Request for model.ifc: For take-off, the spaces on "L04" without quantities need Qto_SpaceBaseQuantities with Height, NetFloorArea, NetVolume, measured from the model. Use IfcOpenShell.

First a look at what the model holds.

```python
import ifcopenshell
import ifcopenshell.util.element
import ifcopenshell.util.unit

model = ifcopenshell.open("model.ifc")
print(model.schema)
for unit_type in ("LENGTHUNIT", "AREAUNIT", "VOLUMEUNIT"):
    print(unit_type, ifcopenshell.util.unit.calculate_unit_scale(model, unit_type))
storey = next(s for s in model.by_type("IfcBuildingStorey") if s.Name == "L04")
spaces = [e for e in ifcopenshell.util.element.get_decomposition(storey) if e.is_a("IfcSpace")]
for e in sorted(spaces, key=lambda e: e.id()):
    print(e.id(), e.is_a(), e.Name, list(ifcopenshell.util.element.get_psets(e, qtos_only=True)), sep=" | ")
```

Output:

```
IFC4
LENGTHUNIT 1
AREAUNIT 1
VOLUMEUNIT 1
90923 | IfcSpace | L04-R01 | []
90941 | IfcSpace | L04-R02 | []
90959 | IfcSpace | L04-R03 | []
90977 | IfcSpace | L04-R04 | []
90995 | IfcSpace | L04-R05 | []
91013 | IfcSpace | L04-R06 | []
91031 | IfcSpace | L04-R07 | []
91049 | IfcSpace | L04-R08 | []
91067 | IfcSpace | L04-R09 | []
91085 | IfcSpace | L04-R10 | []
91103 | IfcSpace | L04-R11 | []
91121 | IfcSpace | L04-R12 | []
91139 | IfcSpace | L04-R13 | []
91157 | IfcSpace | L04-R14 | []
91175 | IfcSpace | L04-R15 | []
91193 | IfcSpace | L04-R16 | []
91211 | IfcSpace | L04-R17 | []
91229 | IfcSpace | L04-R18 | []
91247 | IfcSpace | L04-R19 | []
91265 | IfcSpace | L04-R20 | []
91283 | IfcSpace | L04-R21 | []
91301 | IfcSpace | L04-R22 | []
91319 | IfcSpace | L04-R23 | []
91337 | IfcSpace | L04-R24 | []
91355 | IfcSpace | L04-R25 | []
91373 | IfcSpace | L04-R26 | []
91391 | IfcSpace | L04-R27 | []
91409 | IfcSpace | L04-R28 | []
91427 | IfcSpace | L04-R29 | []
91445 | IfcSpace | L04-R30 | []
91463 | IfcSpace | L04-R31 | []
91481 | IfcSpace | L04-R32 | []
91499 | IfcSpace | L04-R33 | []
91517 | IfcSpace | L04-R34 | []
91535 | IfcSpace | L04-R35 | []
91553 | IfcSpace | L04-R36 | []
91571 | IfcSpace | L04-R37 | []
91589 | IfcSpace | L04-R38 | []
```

```python
import ifcopenshell
import ifcopenshell.api.pset
import ifcopenshell.geom
import ifcopenshell.util.element
import ifcopenshell.util.shape
import ifcopenshell.util.unit

model = ifcopenshell.open("model.ifc")
unit_scale = ifcopenshell.util.unit.calculate_unit_scale(model)
area_scale = ifcopenshell.util.unit.calculate_unit_scale(model, "AREAUNIT")
volume_scale = ifcopenshell.util.unit.calculate_unit_scale(model, "VOLUMEUNIT")
settings = ifcopenshell.geom.settings()

storey = next(s for s in model.by_type("IfcBuildingStorey") if s.Name == "L04")
spaces = [e for e in ifcopenshell.util.element.get_decomposition(storey) if e.is_a("IfcSpace")]

for e in sorted(spaces, key=lambda e: e.id()):
    if ifcopenshell.util.element.get_psets(e, qtos_only=True, should_inherit=False):
        continue
    # Geometry comes back in metres, in the element's own axes.
    shape = ifcopenshell.geom.create_shape(settings, e)
    values = {
        "Height": ifcopenshell.util.shape.get_z(shape.geometry) / unit_scale,
        "NetFloorArea": ifcopenshell.util.shape.get_footprint_area(shape.geometry) / area_scale,
        "NetVolume": ifcopenshell.util.shape.get_volume(shape.geometry) / volume_scale,
    }
    qto = ifcopenshell.api.pset.add_qto(model, product=e, name="Qto_SpaceBaseQuantities")
    ifcopenshell.api.pset.edit_qto(model, qto=qto, properties=values)
    print(e.id(), {k: round(v, 3) for k, v in values.items()})

model.write("model_rev.ifc")
```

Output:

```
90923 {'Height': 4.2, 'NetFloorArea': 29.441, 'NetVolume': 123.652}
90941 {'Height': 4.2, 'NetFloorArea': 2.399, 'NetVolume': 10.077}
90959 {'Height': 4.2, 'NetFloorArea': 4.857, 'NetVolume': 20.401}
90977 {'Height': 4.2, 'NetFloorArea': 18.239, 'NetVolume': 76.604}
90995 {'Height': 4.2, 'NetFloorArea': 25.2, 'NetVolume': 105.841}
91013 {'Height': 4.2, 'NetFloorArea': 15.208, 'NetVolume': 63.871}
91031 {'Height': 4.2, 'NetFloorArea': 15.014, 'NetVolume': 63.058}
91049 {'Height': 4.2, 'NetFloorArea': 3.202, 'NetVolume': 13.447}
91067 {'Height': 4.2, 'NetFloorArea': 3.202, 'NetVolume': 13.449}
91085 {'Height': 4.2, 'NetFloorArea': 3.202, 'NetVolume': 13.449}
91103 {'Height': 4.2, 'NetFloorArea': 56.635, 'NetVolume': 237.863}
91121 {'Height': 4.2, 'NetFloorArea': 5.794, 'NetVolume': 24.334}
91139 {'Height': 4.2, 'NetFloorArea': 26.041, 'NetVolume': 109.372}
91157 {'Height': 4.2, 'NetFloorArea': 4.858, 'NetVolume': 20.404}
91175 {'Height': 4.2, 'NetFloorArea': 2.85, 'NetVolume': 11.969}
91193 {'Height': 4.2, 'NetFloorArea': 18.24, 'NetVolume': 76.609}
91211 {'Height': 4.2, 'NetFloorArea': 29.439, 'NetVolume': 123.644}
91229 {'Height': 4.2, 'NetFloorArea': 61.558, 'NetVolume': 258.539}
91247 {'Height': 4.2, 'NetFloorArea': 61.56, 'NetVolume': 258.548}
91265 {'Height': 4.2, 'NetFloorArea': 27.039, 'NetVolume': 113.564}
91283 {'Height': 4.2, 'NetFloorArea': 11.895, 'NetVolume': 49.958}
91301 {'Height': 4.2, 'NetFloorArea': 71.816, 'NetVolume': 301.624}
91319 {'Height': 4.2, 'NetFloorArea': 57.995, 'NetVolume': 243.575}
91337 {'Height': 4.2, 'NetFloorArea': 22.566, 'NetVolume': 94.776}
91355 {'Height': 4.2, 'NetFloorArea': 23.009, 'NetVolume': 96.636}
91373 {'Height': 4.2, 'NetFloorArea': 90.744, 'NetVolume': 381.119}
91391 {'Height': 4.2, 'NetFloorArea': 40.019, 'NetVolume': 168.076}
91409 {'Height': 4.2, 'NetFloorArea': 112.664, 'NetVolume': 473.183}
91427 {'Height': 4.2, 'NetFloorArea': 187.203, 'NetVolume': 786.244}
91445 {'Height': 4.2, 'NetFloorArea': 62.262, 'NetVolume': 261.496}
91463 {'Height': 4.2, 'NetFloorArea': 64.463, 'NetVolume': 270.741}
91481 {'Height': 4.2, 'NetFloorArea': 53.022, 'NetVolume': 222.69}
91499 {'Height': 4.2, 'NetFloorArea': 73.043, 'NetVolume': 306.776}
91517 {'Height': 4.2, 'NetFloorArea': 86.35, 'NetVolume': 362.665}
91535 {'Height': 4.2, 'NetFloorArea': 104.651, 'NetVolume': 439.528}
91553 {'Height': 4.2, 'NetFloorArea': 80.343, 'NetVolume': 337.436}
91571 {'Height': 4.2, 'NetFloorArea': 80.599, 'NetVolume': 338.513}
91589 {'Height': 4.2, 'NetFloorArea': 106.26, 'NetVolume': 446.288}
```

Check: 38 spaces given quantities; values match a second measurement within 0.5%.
